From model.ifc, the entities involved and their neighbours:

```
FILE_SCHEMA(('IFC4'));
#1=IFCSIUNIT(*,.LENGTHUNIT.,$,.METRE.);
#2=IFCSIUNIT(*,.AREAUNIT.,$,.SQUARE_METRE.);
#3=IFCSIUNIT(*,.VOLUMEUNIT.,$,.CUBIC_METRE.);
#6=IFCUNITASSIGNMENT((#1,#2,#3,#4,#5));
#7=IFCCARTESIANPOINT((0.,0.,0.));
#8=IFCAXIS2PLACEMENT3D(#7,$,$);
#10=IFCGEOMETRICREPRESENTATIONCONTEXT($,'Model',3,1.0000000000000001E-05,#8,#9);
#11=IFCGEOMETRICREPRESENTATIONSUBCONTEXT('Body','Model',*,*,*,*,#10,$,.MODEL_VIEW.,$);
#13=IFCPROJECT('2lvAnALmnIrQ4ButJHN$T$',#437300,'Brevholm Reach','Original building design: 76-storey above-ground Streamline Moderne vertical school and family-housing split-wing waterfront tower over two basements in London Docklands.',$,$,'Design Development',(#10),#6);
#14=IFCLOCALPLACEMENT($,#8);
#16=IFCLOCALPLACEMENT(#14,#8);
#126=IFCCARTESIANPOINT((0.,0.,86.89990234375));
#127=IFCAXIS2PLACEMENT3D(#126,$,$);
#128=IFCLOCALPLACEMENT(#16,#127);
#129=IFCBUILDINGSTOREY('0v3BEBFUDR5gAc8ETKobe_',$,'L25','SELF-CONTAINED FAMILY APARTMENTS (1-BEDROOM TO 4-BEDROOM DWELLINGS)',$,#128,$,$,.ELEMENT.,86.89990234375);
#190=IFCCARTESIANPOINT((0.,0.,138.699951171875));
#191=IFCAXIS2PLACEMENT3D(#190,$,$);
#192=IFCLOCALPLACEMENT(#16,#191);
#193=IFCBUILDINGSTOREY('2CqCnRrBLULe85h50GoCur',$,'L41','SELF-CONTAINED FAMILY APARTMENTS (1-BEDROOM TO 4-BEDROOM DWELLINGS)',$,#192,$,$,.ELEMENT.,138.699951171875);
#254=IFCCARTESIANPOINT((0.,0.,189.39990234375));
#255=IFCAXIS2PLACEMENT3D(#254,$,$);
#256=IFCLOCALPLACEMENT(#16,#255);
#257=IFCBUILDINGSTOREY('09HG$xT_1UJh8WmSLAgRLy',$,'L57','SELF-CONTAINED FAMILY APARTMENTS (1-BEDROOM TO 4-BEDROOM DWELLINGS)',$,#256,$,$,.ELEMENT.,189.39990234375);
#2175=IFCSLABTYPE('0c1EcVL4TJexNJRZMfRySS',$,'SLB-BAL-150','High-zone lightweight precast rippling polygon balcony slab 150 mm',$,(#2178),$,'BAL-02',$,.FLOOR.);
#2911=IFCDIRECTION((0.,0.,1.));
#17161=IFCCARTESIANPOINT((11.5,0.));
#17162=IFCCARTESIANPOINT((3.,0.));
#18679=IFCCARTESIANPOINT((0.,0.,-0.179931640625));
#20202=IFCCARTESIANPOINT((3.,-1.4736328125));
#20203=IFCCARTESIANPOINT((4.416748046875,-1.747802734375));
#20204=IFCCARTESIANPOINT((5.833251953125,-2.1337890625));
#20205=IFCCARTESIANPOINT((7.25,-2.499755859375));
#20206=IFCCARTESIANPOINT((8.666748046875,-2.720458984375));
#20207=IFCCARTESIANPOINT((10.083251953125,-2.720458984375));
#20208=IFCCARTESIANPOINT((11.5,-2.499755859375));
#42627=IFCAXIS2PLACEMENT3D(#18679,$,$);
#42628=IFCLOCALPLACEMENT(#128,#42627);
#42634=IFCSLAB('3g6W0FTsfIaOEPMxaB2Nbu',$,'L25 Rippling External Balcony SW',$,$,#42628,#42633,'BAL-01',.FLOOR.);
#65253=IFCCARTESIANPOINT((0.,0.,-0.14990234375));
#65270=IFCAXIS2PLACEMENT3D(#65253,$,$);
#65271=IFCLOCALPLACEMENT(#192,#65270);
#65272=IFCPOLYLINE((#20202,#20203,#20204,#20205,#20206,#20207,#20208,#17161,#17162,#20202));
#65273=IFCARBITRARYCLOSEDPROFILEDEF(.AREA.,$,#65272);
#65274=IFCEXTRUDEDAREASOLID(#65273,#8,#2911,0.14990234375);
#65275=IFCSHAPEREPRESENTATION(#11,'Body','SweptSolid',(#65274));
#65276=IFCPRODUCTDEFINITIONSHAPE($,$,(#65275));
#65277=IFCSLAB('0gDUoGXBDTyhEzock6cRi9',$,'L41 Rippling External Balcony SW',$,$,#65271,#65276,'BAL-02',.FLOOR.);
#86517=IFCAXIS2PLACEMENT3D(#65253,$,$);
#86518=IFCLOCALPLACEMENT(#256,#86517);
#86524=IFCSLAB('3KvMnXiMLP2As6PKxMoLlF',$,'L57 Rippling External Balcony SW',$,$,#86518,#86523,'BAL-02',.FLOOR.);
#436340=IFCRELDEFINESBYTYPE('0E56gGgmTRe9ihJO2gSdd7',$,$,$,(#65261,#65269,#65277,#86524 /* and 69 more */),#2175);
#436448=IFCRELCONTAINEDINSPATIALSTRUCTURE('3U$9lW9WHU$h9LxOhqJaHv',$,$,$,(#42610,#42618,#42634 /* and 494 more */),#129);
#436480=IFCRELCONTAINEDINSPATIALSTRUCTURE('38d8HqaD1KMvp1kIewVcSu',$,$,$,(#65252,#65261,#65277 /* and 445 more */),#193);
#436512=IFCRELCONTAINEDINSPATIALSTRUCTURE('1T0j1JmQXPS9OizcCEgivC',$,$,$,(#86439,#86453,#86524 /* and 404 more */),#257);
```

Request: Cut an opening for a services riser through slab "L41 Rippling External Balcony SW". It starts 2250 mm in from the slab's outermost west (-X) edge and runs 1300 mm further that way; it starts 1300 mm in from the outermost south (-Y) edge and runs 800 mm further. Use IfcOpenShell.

```python
import numpy as np
import ifcopenshell
import ifcopenshell.api.feature
import ifcopenshell.api.geometry
import ifcopenshell.api.root
import ifcopenshell.geom
import ifcopenshell.util.placement
import ifcopenshell.util.representation
import ifcopenshell.util.shape
import ifcopenshell.util.unit

model = ifcopenshell.open("model.ifc")
unit_scale = ifcopenshell.util.unit.calculate_unit_scale(model)
settings = ifcopenshell.geom.settings()


def volume(element):
    """Net volume in cubic metres, openings subtracted."""
    shape = ifcopenshell.geom.create_shape(settings, element)
    return ifcopenshell.util.shape.get_volume(shape.geometry)


slab = model.by_id(65277)
before = volume(slab)

# Extent in the slab's own axes, in metres. The edges named are its -X and -Y sides.
slab_shape = ifcopenshell.geom.create_shape(settings, slab)
vertices = ifcopenshell.util.shape.get_vertices(slab_shape.geometry)
x_min, y_min, bottom = vertices.min(axis=0)
top = vertices[:, 2].max()

opening = ifcopenshell.api.root.create_entity(model, ifc_class="IfcOpeningElement", name="Services riser opening", predefined_type="OPENING")
context = ifcopenshell.util.representation.get_context(model, "Model", "Body", "MODEL_VIEW")
width, depth = 1.3, 0.8
outline = [(0.0, 0.0), (width, 0.0), (width, depth), (0.0, depth), (0.0, 0.0)]
# Overshoot both faces by 50 mm so the cut is clean.
shape = ifcopenshell.api.geometry.add_slab_representation(
    model, context=context, depth=top - bottom + 0.1, polyline=outline
)
ifcopenshell.api.geometry.assign_representation(model, product=opening, representation=shape)

matrix = ifcopenshell.util.placement.get_local_placement(slab.ObjectPlacement)
matrix[:, 3] = matrix @ np.append(np.array([x_min + 2.25, y_min + 1.3, bottom - 0.05]) / unit_scale, 1.0)
ifcopenshell.api.geometry.edit_object_placement(model, product=opening, matrix=matrix, is_si=False)
ifcopenshell.api.feature.add_feature(model, feature=opening, element=slab)

after = volume(slab)

print(f"slab volume {before:.3f} -> {after:.3f} m3")

model.write("model_edited.ifc")
```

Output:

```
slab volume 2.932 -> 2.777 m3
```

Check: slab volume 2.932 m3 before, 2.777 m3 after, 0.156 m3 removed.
